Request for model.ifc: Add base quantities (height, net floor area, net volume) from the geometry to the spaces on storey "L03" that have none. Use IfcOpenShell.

First a look at what the model holds.

```python
import ifcopenshell
import ifcopenshell.util.element
import ifcopenshell.util.unit

model = ifcopenshell.open("model.ifc")
print(model.schema)
for unit_type in ("LENGTHUNIT", "AREAUNIT", "VOLUMEUNIT"):
    print(unit_type, ifcopenshell.util.unit.calculate_unit_scale(model, unit_type))
storey = next(s for s in model.by_type("IfcBuildingStorey") if s.Name == "L03")
spaces = [e for e in ifcopenshell.util.element.get_decomposition(storey) if e.is_a("IfcSpace")]
for e in sorted(spaces, key=lambda e: e.id()):
    print(e.id(), e.is_a(), e.Name, list(ifcopenshell.util.element.get_psets(e, qtos_only=True)), sep=" | ")
```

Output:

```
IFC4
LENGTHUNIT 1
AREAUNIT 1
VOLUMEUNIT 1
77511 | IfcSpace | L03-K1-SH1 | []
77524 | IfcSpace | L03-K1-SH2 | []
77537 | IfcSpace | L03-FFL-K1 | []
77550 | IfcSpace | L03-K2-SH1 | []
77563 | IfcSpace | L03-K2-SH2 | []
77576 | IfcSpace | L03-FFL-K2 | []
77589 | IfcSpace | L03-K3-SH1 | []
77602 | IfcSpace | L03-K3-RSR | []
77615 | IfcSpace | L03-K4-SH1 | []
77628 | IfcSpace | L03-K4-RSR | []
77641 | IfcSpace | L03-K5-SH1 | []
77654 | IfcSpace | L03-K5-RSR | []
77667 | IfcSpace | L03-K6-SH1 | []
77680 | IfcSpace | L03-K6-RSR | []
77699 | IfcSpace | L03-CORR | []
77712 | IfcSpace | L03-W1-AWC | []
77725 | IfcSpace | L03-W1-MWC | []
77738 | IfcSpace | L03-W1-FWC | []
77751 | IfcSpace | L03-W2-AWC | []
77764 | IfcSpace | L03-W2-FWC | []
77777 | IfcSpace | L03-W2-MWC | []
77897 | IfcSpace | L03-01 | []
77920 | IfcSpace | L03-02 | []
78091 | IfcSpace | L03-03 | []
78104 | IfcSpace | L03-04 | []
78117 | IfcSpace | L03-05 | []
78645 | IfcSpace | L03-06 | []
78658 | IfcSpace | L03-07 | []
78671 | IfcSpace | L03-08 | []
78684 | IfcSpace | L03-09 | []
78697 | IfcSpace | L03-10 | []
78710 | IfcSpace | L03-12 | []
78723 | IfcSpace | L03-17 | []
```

```python
import ifcopenshell
import ifcopenshell.api.pset
import ifcopenshell.geom
import ifcopenshell.util.element
import ifcopenshell.util.shape
import ifcopenshell.util.unit

model = ifcopenshell.open("model.ifc")
unit_scale = ifcopenshell.util.unit.calculate_unit_scale(model)
area_scale = ifcopenshell.util.unit.calculate_unit_scale(model, "AREAUNIT")
volume_scale = ifcopenshell.util.unit.calculate_unit_scale(model, "VOLUMEUNIT")
settings = ifcopenshell.geom.settings()

storey = next(s for s in model.by_type("IfcBuildingStorey") if s.Name == "L03")
spaces = [e for e in ifcopenshell.util.element.get_decomposition(storey) if e.is_a("IfcSpace")]

for e in sorted(spaces, key=lambda e: e.id()):
    if ifcopenshell.util.element.get_psets(e, qtos_only=True, should_inherit=False):
        continue
    # Geometry comes back in metres, in the element's own axes.
    shape = ifcopenshell.geom.create_shape(settings, e)
    values = {
        "Height": ifcopenshell.util.shape.get_z(shape.geometry) / unit_scale,
        "NetFloorArea": ifcopenshell.util.shape.get_footprint_area(shape.geometry) / area_scale,
        "NetVolume": ifcopenshell.util.shape.get_volume(shape.geometry) / volume_scale,
    }
    qto = ifcopenshell.api.pset.add_qto(model, product=e, name="Qto_SpaceBaseQuantities")
    ifcopenshell.api.pset.edit_qto(model, qto=qto, properties=values)
    print(e.id(), {k: round(v, 3) for k, v in values.items()})

model.write("model_v2.ifc")
```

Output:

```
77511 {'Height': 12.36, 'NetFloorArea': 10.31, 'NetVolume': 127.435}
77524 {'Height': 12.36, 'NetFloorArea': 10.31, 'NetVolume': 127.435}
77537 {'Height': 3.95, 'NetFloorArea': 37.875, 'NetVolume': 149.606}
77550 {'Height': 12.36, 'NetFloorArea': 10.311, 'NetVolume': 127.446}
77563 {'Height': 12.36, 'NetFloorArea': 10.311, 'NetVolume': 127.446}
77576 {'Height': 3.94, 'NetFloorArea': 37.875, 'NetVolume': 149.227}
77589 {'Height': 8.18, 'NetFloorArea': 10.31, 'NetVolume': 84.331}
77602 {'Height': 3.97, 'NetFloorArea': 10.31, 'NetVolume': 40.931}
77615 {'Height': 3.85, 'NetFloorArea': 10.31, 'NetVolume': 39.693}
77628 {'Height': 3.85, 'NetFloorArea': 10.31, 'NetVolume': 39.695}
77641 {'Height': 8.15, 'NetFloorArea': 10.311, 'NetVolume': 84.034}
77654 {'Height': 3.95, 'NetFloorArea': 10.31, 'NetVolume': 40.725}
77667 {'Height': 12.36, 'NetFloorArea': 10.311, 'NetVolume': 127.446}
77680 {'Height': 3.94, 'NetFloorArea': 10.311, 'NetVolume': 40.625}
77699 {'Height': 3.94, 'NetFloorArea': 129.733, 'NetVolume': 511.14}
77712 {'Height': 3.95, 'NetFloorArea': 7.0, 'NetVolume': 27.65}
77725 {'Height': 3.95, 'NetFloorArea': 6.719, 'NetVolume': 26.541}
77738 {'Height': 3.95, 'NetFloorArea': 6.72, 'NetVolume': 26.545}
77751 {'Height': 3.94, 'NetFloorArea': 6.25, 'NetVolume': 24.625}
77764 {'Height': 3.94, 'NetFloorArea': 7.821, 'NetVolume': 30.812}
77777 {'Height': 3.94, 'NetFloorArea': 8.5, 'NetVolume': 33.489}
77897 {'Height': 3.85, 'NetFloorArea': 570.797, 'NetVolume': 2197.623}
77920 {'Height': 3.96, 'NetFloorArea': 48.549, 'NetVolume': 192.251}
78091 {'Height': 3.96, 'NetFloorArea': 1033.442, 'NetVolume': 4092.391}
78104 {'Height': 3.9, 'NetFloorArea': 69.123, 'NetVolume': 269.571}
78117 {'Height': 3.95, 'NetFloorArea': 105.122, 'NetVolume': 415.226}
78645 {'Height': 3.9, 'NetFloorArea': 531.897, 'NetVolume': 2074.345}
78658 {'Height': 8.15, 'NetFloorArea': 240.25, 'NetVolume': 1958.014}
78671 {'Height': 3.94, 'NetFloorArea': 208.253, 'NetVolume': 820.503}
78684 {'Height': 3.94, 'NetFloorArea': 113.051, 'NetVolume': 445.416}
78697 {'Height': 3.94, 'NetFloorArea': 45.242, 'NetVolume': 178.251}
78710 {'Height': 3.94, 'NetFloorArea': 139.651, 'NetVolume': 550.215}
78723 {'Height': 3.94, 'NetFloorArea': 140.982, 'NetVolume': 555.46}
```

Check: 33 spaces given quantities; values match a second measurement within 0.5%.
